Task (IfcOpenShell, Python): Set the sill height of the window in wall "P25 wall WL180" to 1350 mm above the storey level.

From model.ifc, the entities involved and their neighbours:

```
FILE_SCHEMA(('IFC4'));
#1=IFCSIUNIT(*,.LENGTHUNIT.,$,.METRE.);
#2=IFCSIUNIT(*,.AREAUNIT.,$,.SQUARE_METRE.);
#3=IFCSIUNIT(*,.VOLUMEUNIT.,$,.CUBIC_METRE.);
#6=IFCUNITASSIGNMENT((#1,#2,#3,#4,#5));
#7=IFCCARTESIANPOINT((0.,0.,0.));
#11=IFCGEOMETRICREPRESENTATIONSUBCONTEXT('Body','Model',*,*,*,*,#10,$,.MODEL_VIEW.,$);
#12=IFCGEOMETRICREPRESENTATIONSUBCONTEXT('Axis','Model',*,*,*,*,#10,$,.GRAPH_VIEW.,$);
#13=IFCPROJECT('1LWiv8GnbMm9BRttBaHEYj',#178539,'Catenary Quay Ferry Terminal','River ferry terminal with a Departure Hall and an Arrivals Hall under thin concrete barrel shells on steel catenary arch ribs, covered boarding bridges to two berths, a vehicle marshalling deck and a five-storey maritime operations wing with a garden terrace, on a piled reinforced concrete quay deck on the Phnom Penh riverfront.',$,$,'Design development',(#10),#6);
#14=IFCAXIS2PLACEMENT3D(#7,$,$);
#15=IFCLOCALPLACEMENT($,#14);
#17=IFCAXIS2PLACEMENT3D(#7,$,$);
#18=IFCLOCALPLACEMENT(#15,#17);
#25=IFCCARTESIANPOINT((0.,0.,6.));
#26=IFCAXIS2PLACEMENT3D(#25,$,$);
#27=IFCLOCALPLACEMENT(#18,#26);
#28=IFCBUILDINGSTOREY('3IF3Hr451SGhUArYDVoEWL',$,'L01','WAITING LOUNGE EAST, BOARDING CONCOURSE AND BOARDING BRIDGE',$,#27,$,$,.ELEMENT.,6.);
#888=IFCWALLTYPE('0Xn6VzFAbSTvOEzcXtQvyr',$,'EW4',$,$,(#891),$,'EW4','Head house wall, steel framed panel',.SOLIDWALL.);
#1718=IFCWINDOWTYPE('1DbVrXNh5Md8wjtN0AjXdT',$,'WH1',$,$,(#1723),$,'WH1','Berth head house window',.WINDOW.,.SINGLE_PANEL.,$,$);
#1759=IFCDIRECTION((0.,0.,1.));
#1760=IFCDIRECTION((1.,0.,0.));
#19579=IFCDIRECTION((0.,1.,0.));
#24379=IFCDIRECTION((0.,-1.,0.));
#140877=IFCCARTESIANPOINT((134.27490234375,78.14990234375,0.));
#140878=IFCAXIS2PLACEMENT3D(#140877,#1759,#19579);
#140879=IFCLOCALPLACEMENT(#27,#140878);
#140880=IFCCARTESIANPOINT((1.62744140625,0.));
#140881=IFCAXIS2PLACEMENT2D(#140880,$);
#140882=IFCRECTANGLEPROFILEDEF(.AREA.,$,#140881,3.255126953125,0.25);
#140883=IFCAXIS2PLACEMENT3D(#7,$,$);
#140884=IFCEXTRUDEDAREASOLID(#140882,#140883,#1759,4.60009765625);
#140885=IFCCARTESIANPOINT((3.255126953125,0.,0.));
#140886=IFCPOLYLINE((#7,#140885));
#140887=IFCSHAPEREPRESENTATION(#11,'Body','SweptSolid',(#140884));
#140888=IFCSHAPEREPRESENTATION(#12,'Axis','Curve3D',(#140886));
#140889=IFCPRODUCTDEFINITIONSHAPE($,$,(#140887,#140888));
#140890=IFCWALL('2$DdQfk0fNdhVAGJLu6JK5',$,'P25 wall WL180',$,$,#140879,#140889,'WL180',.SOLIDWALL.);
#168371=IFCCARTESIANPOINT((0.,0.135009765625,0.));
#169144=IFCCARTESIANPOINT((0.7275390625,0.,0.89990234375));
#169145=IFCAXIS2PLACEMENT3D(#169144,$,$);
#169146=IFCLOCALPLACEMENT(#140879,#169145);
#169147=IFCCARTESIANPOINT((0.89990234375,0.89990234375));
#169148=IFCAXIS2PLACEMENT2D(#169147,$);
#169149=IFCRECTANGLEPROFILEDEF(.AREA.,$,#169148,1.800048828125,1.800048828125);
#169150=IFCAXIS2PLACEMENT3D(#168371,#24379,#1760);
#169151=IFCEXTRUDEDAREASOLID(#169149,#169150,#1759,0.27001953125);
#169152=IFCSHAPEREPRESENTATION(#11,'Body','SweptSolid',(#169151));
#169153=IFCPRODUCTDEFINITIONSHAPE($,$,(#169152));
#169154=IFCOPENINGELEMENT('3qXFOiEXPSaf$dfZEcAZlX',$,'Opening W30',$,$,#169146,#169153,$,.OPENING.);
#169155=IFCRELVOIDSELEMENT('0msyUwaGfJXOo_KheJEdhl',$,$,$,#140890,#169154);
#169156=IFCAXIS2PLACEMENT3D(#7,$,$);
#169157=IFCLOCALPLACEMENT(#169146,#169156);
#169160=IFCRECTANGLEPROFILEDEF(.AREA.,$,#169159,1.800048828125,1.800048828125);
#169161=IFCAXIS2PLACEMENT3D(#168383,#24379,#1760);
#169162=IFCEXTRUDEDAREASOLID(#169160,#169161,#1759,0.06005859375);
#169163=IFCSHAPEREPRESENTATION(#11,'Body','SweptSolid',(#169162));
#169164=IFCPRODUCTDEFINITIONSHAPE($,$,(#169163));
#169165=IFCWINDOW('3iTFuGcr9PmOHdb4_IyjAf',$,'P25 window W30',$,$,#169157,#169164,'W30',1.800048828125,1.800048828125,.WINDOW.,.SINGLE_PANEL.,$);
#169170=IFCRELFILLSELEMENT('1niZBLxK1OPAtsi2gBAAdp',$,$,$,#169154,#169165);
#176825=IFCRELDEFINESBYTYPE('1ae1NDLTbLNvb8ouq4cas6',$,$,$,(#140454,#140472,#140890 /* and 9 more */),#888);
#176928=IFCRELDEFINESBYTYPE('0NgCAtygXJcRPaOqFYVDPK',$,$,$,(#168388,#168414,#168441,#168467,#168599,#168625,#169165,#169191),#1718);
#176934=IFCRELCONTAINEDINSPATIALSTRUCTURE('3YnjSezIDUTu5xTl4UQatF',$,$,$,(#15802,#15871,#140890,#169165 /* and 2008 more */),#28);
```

```python
import numpy as np
import ifcopenshell
import ifcopenshell.api.geometry
import ifcopenshell.geom
import ifcopenshell.util.element
import ifcopenshell.util.placement
import ifcopenshell.util.shape
import ifcopenshell.util.unit

model = ifcopenshell.open("model.ifc")
unit_scale = ifcopenshell.util.unit.calculate_unit_scale(model)

window = model.by_guid("3iTFuGcr9PmOHdb4_IyjAf")
opening = window.FillsVoids[0].RelatingOpeningElement
storey = ifcopenshell.util.element.get_container(window, ifc_class="IfcBuildingStorey")
level = ifcopenshell.util.placement.get_local_placement(storey.ObjectPlacement)[2, 3]

# The opening's origin need not be at the sill, so measure its lowest point.
shape = ifcopenshell.geom.create_shape(ifcopenshell.geom.settings(), opening)
bottom = ifcopenshell.util.shape.get_shape_bottom_elevation(shape, shape.geometry) / unit_scale
dz = level + 1.35 / unit_scale - bottom

shift = np.array([0.0, 0.0, dz])
# The window is placed relative to its opening, so it follows when the opening moves.
matrix = ifcopenshell.util.placement.get_local_placement(opening.ObjectPlacement)
matrix[:3, 3] += shift
ifcopenshell.api.geometry.edit_object_placement(
    model, product=opening, matrix=matrix, is_si=False, should_transform_children=True
)

print(f"moved by {dz * unit_scale:+.3f} m")

model.write("model_rev.ifc")
```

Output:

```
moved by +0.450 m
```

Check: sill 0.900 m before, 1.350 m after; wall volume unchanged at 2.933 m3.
